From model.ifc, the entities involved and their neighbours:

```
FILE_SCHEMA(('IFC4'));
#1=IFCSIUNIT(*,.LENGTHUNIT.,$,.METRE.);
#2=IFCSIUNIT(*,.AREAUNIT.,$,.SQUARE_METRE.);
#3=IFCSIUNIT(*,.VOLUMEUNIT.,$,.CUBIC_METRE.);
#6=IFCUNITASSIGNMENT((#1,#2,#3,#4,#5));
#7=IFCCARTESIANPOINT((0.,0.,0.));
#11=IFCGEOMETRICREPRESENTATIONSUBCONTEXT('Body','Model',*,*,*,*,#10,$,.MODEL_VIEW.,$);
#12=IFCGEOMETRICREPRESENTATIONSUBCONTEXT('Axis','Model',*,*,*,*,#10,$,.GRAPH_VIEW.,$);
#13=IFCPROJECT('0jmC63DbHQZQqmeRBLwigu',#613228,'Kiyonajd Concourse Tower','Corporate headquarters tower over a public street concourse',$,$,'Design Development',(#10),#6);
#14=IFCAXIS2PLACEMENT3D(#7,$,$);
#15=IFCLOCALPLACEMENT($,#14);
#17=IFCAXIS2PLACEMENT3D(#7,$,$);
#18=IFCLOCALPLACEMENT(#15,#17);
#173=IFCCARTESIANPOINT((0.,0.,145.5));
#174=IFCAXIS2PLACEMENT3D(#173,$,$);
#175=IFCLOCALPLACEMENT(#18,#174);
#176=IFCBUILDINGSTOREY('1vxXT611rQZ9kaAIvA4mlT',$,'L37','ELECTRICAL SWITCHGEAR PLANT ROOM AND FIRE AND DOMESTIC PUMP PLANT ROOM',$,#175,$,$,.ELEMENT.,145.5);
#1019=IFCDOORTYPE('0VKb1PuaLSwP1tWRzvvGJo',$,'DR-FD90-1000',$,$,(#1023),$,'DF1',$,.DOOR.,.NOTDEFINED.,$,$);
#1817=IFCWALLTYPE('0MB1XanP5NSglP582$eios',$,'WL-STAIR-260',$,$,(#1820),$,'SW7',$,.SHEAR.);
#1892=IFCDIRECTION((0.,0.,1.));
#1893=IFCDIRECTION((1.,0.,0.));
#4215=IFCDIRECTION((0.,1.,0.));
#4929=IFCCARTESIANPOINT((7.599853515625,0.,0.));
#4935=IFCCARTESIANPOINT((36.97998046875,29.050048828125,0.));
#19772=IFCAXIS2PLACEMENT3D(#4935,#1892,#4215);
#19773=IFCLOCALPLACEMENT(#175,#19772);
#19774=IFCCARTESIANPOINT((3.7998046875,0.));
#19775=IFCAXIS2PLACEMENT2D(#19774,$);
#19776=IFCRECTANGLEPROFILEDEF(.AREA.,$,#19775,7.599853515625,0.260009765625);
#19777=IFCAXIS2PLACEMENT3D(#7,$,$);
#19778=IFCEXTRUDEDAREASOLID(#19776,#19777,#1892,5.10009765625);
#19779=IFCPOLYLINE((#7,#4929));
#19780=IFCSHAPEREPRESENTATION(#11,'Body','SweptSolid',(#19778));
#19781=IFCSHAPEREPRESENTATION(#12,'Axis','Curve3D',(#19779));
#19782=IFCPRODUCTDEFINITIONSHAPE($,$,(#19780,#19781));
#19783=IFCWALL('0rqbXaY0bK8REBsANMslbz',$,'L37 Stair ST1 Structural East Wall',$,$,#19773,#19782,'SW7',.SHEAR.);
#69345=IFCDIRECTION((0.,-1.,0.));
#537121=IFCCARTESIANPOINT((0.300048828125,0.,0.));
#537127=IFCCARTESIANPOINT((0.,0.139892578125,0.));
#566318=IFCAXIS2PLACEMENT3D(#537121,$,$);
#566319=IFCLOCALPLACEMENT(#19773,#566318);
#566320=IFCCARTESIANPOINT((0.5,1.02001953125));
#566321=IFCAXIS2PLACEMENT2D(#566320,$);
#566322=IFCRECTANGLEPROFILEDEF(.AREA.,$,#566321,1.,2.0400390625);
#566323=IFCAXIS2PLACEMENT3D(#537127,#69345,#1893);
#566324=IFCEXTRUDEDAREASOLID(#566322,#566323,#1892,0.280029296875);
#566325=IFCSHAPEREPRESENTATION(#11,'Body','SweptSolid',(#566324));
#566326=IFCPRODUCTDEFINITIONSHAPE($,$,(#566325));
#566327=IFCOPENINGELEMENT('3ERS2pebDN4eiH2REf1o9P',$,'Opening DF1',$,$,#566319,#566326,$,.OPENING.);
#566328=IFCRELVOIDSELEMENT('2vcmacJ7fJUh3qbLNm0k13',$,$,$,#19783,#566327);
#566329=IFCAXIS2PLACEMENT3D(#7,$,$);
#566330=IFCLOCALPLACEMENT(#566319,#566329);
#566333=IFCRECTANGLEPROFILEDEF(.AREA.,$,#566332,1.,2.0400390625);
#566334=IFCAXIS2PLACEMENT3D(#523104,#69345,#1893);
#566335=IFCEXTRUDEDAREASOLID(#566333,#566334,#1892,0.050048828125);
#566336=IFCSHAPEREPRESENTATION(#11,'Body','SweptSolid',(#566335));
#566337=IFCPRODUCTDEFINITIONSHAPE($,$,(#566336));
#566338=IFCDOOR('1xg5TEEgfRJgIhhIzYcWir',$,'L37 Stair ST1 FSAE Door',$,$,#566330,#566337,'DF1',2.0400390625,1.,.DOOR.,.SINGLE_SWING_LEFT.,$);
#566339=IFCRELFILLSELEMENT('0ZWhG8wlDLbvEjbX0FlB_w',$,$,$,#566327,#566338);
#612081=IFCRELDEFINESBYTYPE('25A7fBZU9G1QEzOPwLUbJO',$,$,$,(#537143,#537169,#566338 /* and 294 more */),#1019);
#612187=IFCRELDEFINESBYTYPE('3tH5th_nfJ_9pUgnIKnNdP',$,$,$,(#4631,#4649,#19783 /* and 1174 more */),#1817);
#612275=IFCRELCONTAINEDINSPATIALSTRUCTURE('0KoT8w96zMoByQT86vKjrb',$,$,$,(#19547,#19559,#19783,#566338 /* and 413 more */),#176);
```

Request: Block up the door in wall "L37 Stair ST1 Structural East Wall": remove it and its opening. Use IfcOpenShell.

```python
import ifcopenshell
import ifcopenshell.api.feature
import ifcopenshell.api.root
import ifcopenshell.geom
import ifcopenshell.util.shape

model = ifcopenshell.open("model.ifc")
settings = ifcopenshell.geom.settings()


def volume(element):
    """Net volume in cubic metres, openings subtracted."""
    shape = ifcopenshell.geom.create_shape(settings, element)
    return ifcopenshell.util.shape.get_volume(shape.geometry)


door = model.by_guid("1xg5TEEgfRJgIhhIzYcWir")
opening = door.FillsVoids[0].RelatingOpeningElement
wall = opening.VoidsElements[0].RelatingBuildingElement
before = volume(wall)

ifcopenshell.api.root.remove_product(model, product=door)
ifcopenshell.api.feature.remove_feature(model, feature=opening)

after = volume(wall)

print(f"wall volume {before:.3f} -> {after:.3f} m3")

model.write("model_rev.ifc")
```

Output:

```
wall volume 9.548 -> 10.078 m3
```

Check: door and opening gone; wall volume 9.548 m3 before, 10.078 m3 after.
